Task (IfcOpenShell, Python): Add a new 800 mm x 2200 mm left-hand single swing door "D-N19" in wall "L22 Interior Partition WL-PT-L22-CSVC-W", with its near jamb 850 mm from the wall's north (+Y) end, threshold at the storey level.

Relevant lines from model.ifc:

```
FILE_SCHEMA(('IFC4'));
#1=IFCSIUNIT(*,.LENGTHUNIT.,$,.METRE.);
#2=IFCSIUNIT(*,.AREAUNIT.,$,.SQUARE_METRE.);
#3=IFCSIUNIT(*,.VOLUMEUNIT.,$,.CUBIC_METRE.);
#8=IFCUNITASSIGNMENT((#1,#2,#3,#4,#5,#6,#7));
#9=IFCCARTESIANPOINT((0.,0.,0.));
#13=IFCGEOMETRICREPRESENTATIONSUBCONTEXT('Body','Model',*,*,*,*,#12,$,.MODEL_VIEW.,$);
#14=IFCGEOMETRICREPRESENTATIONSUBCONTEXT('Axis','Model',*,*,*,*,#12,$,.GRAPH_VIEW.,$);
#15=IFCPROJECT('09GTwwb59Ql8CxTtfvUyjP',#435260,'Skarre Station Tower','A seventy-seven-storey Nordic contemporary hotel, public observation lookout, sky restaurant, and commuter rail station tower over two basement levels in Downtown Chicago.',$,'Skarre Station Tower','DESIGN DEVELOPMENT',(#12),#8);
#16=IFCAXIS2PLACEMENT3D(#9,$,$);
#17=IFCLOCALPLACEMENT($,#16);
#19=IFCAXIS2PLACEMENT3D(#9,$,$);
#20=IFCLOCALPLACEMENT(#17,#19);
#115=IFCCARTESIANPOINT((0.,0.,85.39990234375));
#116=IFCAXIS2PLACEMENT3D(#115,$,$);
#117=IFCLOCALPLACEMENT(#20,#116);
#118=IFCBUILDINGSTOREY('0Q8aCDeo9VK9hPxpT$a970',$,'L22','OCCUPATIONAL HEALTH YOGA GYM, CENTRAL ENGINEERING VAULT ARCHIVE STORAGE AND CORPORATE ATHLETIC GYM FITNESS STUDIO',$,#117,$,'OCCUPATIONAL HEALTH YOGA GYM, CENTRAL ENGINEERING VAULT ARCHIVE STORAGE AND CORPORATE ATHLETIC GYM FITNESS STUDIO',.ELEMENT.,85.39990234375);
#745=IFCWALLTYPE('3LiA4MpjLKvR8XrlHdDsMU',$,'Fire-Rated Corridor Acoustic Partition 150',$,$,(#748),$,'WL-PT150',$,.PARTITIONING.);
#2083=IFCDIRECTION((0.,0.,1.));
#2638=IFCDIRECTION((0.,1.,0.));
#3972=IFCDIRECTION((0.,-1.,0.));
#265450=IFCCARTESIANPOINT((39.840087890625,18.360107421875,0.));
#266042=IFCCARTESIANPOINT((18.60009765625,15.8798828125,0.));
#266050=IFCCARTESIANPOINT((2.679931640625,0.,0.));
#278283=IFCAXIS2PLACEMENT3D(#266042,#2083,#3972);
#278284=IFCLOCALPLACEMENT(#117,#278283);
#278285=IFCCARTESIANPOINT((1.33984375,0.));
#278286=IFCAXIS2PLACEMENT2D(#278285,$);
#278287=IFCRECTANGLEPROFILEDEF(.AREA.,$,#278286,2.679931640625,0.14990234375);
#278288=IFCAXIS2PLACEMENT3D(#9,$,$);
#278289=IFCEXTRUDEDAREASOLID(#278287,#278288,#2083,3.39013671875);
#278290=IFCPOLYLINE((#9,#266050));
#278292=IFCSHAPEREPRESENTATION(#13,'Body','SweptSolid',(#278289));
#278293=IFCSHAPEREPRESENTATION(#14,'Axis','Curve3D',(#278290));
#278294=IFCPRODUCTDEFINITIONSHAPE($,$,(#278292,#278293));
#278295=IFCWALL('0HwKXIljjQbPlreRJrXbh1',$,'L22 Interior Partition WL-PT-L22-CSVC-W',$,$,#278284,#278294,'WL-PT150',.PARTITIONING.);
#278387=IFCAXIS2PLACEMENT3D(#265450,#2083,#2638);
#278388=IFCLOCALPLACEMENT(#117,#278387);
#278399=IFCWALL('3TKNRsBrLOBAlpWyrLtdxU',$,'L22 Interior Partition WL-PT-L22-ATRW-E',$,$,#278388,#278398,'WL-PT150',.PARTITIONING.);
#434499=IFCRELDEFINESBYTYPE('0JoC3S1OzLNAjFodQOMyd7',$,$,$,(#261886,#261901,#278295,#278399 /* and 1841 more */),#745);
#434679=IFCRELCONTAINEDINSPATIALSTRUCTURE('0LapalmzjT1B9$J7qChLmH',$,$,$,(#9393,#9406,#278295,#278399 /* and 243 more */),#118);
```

```python
import numpy as np
import ifcopenshell
import ifcopenshell.api.feature
import ifcopenshell.api.geometry
import ifcopenshell.api.root
import ifcopenshell.api.spatial
import ifcopenshell.geom
import ifcopenshell.util.element
import ifcopenshell.util.placement
import ifcopenshell.util.representation
import ifcopenshell.util.shape
import ifcopenshell.util.unit

model = ifcopenshell.open("model.ifc")
unit_scale = ifcopenshell.util.unit.calculate_unit_scale(model)
settings = ifcopenshell.geom.settings()


def volume(element):
    """Net volume in cubic metres, openings subtracted."""
    shape = ifcopenshell.geom.create_shape(settings, element)
    return ifcopenshell.util.shape.get_volume(shape.geometry)


wall = model.by_guid("0HwKXIljjQbPlreRJrXbh1")
storey = ifcopenshell.util.element.get_container(wall, ifc_class="IfcBuildingStorey")
context = ifcopenshell.util.representation.get_context(model, "Model", "Body", "MODEL_VIEW")
before = volume(wall)

width, height, from_end, sill = 0.8, 2.2, 0.85, 0.0  # metres

# The wall runs along its own X axis, and the end named is its -X end.
wall_shape = ifcopenshell.geom.create_shape(settings, wall)
x, y, z = ifcopenshell.util.shape.get_vertices(wall_shape.geometry).T
start = x.min() + from_end
face, thickness = float(y.min()), float(y.max() - y.min())
wall_matrix = ifcopenshell.util.placement.get_local_placement(wall.ObjectPlacement)
level = ifcopenshell.util.placement.get_local_placement(storey.ObjectPlacement)[2, 3]


def in_wall(x, y):
    """Placement at x, y metres in the wall's axes, at sill height."""
    matrix = wall_matrix.copy()
    matrix[:, 3] = wall_matrix @ np.array([x / unit_scale, y / unit_scale, 0.0, 1.0])
    matrix[2, 3] = level + sill / unit_scale
    return matrix


# Opening: a box that overshoots both wall faces by 50 mm.
opening = ifcopenshell.api.root.create_entity(model, ifc_class="IfcOpeningElement", predefined_type="OPENING")
box = ifcopenshell.api.geometry.add_wall_representation(
    model, context=context, length=width, height=height, thickness=thickness + 0.1
)
ifcopenshell.api.geometry.assign_representation(model, product=opening, representation=box)
ifcopenshell.api.geometry.edit_object_placement(model, product=opening, matrix=in_wall(start, face - 0.05), is_si=False)
ifcopenshell.api.feature.add_feature(model, feature=opening, element=wall)

door = ifcopenshell.api.root.create_entity(model, ifc_class="IfcDoor", name="D-N19", predefined_type="DOOR")
door.OverallWidth, door.OverallHeight = width / unit_scale, height / unit_scale
door.OperationType = "SINGLE_SWING_LEFT"
body = ifcopenshell.api.geometry.add_door_representation(
    model,
    context=context,
    overall_width=door.OverallWidth,
    overall_height=door.OverallHeight,
    operation_type="SINGLE_SWING_LEFT",
    lining_properties={"LiningDepth": thickness / unit_scale, "ThresholdDepth": thickness / unit_scale},
)
ifcopenshell.api.geometry.assign_representation(model, product=door, representation=body)
ifcopenshell.api.spatial.assign_container(model, products=[door], relating_structure=storey)
ifcopenshell.api.feature.add_filling(model, opening=opening, element=door)

# The lining spans the wall, so the door starts at the wall face.
ifcopenshell.api.geometry.edit_object_placement(model, product=door, matrix=in_wall(start, face), is_si=False)

after = volume(wall)

print(f"wall volume {before:.3f} -> {after:.3f} m3")

model.write("model_updated.ifc")
```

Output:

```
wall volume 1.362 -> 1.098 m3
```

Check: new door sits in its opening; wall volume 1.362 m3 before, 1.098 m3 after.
